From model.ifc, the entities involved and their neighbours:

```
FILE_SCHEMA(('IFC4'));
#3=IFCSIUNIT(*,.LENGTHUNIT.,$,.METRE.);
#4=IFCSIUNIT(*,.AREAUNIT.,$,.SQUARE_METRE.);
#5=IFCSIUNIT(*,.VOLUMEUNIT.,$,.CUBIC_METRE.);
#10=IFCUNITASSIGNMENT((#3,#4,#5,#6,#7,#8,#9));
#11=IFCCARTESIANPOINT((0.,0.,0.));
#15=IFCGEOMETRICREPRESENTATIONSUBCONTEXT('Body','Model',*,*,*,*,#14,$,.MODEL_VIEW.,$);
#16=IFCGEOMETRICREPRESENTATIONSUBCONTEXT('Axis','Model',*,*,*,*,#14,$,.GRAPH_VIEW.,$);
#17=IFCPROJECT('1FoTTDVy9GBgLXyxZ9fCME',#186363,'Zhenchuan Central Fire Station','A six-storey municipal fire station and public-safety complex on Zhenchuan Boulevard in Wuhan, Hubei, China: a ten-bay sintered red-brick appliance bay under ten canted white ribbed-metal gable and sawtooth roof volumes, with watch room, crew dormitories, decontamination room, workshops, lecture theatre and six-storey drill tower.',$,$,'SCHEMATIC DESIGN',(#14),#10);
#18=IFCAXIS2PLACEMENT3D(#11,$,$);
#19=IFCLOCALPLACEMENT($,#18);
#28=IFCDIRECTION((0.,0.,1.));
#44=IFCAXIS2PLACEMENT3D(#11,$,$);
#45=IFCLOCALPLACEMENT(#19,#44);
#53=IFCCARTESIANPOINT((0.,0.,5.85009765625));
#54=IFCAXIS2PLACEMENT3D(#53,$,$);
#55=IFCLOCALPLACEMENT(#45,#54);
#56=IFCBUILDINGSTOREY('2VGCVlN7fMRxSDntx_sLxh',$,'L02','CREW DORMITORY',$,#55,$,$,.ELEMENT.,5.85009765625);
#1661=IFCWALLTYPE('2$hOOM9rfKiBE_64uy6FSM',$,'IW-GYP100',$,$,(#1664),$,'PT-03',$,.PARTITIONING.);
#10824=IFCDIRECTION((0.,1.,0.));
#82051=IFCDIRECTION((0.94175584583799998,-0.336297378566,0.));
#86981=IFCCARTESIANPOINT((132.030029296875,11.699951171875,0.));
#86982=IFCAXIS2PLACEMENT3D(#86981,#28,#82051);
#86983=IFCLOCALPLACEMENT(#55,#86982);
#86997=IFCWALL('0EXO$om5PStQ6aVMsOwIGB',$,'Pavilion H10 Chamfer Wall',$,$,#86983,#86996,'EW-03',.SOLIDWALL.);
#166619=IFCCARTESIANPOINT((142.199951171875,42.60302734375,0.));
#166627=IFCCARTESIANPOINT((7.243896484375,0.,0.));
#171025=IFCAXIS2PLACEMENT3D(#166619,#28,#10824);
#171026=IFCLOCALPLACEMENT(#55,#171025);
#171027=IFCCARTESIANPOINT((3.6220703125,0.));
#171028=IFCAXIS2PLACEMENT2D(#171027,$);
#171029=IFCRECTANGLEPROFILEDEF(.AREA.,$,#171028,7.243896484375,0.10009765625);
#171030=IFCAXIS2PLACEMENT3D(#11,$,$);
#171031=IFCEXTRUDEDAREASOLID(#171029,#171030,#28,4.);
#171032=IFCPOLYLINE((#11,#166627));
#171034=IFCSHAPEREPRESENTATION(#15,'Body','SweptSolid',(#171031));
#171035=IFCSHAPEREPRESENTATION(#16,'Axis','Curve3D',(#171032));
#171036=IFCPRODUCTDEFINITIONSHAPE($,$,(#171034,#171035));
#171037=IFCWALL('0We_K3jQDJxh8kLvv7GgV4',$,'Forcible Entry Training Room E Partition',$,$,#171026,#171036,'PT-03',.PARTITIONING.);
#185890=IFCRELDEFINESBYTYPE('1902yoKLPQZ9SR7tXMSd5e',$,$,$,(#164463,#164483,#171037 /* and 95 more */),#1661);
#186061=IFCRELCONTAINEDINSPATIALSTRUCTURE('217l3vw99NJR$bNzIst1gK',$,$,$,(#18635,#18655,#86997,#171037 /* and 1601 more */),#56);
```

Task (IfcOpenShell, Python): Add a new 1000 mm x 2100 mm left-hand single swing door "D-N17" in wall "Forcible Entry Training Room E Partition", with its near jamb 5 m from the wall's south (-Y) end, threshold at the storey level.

```python
import numpy as np
import ifcopenshell
import ifcopenshell.api.feature
import ifcopenshell.api.geometry
import ifcopenshell.api.root
import ifcopenshell.api.spatial
import ifcopenshell.geom
import ifcopenshell.util.element
import ifcopenshell.util.placement
import ifcopenshell.util.representation
import ifcopenshell.util.shape
import ifcopenshell.util.unit

model = ifcopenshell.open("model.ifc")
unit_scale = ifcopenshell.util.unit.calculate_unit_scale(model)
settings = ifcopenshell.geom.settings()


def volume(element):
    """Net volume in cubic metres, openings subtracted."""
    shape = ifcopenshell.geom.create_shape(settings, element)
    return ifcopenshell.util.shape.get_volume(shape.geometry)


wall = model.by_id(171037)
storey = ifcopenshell.util.element.get_container(wall, ifc_class="IfcBuildingStorey")
context = ifcopenshell.util.representation.get_context(model, "Model", "Body", "MODEL_VIEW")
before = volume(wall)

width, height, from_end, sill = 1, 2.1, 5, 0.0  # metres

# The wall runs along its own X axis, and the end named is its -X end.
wall_shape = ifcopenshell.geom.create_shape(settings, wall)
x, y, z = ifcopenshell.util.shape.get_vertices(wall_shape.geometry).T
start = x.min() + from_end
face, thickness = float(y.min()), float(y.max() - y.min())
wall_matrix = ifcopenshell.util.placement.get_local_placement(wall.ObjectPlacement)
level = ifcopenshell.util.placement.get_local_placement(storey.ObjectPlacement)[2, 3]


def in_wall(x, y):
    """Placement at x, y metres in the wall's axes, at sill height."""
    matrix = wall_matrix.copy()
    matrix[:, 3] = wall_matrix @ np.array([x / unit_scale, y / unit_scale, 0.0, 1.0])
    matrix[2, 3] = level + sill / unit_scale
    return matrix


# Opening: a box that overshoots both wall faces by 50 mm.
opening = ifcopenshell.api.root.create_entity(model, ifc_class="IfcOpeningElement", predefined_type="OPENING")
box = ifcopenshell.api.geometry.add_wall_representation(
    model, context=context, length=width, height=height, thickness=thickness + 0.1
)
ifcopenshell.api.geometry.assign_representation(model, product=opening, representation=box)
ifcopenshell.api.geometry.edit_object_placement(model, product=opening, matrix=in_wall(start, face - 0.05), is_si=False)
ifcopenshell.api.feature.add_feature(model, feature=opening, element=wall)

door = ifcopenshell.api.root.create_entity(model, ifc_class="IfcDoor", name="D-N17", predefined_type="DOOR")
door.OverallWidth, door.OverallHeight = width / unit_scale, height / unit_scale
door.OperationType = "SINGLE_SWING_LEFT"
body = ifcopenshell.api.geometry.add_door_representation(
    model,
    context=context,
    overall_width=door.OverallWidth,
    overall_height=door.OverallHeight,
    operation_type="SINGLE_SWING_LEFT",
    lining_properties={"LiningDepth": thickness / unit_scale, "ThresholdDepth": thickness / unit_scale},
)
ifcopenshell.api.geometry.assign_representation(model, product=door, representation=body)
ifcopenshell.api.spatial.assign_container(model, products=[door], relating_structure=storey)
ifcopenshell.api.feature.add_filling(model, opening=opening, element=door)

# The lining spans the wall, so the door starts at the wall face.
ifcopenshell.api.geometry.edit_object_placement(model, product=door, matrix=in_wall(start, face), is_si=False)

after = volume(wall)

print(f"wall volume {before:.3f} -> {after:.3f} m3")

model.write("model_rev.ifc")
```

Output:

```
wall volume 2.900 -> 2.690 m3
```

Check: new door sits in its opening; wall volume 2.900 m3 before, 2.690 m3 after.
